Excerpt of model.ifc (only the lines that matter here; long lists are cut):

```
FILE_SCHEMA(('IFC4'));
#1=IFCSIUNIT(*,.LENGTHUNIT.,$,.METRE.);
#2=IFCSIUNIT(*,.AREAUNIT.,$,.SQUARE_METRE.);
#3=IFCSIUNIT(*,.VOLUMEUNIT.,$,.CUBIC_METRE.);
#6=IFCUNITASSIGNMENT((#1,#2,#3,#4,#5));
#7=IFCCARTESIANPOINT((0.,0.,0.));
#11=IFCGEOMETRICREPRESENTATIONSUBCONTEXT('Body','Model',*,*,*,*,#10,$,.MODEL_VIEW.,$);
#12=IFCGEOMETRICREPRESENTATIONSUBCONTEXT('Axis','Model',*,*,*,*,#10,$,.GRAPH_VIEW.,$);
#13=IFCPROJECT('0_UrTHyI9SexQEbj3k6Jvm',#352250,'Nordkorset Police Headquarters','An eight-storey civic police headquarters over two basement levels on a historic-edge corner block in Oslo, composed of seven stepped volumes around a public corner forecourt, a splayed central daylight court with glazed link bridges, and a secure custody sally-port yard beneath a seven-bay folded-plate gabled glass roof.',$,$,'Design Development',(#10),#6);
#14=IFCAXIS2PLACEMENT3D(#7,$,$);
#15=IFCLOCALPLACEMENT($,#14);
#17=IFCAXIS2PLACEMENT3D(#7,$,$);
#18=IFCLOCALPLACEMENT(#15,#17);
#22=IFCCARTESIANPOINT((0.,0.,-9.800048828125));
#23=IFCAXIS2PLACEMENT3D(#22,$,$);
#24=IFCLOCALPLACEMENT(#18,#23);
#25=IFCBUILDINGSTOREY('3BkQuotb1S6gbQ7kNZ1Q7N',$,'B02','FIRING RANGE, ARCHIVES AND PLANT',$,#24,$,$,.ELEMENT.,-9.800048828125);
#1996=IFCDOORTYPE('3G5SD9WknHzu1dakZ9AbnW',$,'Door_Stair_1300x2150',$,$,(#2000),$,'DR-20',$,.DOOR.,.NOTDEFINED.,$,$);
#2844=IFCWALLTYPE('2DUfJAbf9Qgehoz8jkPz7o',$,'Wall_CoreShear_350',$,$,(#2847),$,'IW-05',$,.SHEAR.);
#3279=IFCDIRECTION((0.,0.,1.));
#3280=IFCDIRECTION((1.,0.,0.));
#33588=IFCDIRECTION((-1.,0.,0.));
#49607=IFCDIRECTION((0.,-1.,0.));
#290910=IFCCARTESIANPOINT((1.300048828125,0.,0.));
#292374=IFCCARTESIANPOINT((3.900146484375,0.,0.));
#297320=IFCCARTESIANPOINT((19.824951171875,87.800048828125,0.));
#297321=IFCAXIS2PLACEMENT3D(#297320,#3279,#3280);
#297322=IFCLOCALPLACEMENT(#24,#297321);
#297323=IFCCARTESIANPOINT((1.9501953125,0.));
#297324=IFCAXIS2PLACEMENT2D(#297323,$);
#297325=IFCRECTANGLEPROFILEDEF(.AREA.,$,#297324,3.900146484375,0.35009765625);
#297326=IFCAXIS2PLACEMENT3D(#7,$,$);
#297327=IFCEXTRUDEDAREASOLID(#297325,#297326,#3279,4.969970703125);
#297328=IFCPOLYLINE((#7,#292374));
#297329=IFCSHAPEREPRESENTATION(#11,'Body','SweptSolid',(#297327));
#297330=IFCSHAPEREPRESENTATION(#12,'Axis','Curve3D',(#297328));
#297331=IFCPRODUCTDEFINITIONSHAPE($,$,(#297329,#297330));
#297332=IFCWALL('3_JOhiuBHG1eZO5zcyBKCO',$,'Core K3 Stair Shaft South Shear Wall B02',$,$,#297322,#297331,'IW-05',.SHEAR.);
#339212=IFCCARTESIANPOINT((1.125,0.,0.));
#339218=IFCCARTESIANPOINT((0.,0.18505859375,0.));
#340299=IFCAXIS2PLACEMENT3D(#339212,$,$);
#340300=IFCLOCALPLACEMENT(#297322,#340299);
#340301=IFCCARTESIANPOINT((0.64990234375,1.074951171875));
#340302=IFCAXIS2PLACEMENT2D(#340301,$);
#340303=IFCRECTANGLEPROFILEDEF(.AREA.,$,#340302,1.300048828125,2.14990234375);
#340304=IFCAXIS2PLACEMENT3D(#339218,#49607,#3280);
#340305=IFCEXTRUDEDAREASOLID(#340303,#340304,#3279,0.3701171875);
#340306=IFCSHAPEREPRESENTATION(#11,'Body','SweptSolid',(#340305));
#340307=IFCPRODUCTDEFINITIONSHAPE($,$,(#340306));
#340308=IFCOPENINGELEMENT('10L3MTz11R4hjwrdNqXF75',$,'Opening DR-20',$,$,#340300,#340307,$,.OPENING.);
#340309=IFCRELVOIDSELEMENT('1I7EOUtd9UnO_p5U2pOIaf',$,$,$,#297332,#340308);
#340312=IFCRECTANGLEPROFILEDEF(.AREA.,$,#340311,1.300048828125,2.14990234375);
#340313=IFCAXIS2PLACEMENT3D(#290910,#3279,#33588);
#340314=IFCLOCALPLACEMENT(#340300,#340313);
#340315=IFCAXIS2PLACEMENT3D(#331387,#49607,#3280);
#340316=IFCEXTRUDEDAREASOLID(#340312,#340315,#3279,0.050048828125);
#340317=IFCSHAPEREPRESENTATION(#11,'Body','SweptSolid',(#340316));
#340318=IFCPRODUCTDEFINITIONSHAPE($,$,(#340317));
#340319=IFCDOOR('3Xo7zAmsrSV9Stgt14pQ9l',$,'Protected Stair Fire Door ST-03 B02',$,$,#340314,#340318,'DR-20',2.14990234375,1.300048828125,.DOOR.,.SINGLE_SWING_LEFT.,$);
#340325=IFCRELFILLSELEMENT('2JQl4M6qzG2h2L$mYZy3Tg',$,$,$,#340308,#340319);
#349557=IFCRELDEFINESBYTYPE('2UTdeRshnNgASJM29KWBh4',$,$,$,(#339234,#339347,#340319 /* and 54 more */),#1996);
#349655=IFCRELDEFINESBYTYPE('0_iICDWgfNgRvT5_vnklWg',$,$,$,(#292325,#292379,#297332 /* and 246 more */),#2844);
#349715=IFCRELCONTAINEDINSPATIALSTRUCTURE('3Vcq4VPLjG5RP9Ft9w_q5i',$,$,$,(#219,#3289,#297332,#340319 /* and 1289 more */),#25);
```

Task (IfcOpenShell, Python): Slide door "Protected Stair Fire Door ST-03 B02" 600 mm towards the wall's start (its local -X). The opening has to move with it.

```python
import ifcopenshell
import ifcopenshell.api.geometry
import ifcopenshell.util.placement
import ifcopenshell.util.unit

model = ifcopenshell.open("model.ifc")
unit_scale = ifcopenshell.util.unit.calculate_unit_scale(model)

door = model.by_guid("3Xo7zAmsrSV9Stgt14pQ9l")
opening = door.FillsVoids[0].RelatingOpeningElement
wall = opening.VoidsElements[0].RelatingBuildingElement

wall_matrix = ifcopenshell.util.placement.get_local_placement(wall.ObjectPlacement)
shift = wall_matrix[:3, 0] * -0.6 / unit_scale
before = ifcopenshell.util.placement.get_local_placement(door.ObjectPlacement)[:3, 3].copy()

# The door is placed relative to its opening, so it follows when the opening moves.
matrix = ifcopenshell.util.placement.get_local_placement(opening.ObjectPlacement)
matrix[:3, 3] += shift
ifcopenshell.api.geometry.edit_object_placement(
    model, product=opening, matrix=matrix, is_si=False, should_transform_children=True
)

after = ifcopenshell.util.placement.get_local_placement(door.ObjectPlacement)[:3, 3]
print("door moved by", (after - before).round(3) + 0.0)

model.write("model-out.ifc")
```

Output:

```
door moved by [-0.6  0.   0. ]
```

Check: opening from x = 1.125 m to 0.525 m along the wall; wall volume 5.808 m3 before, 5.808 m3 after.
